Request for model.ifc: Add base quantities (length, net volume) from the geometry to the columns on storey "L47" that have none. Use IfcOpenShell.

First a look at what the model holds.

```python
import ifcopenshell
import ifcopenshell.util.element
import ifcopenshell.util.unit

model = ifcopenshell.open("model.ifc")
print(model.schema)
for unit_type in ("LENGTHUNIT", "AREAUNIT", "VOLUMEUNIT"):
    print(unit_type, ifcopenshell.util.unit.calculate_unit_scale(model, unit_type))
storey = next(s for s in model.by_type("IfcBuildingStorey") if s.Name == "L47")
columns = [e for e in ifcopenshell.util.element.get_decomposition(storey) if e.is_a("IfcColumn")]
for e in sorted(columns, key=lambda e: e.id()):
    print(e.id(), e.is_a(), e.Name, list(ifcopenshell.util.element.get_psets(e, qtos_only=True)), sep=" | ")
```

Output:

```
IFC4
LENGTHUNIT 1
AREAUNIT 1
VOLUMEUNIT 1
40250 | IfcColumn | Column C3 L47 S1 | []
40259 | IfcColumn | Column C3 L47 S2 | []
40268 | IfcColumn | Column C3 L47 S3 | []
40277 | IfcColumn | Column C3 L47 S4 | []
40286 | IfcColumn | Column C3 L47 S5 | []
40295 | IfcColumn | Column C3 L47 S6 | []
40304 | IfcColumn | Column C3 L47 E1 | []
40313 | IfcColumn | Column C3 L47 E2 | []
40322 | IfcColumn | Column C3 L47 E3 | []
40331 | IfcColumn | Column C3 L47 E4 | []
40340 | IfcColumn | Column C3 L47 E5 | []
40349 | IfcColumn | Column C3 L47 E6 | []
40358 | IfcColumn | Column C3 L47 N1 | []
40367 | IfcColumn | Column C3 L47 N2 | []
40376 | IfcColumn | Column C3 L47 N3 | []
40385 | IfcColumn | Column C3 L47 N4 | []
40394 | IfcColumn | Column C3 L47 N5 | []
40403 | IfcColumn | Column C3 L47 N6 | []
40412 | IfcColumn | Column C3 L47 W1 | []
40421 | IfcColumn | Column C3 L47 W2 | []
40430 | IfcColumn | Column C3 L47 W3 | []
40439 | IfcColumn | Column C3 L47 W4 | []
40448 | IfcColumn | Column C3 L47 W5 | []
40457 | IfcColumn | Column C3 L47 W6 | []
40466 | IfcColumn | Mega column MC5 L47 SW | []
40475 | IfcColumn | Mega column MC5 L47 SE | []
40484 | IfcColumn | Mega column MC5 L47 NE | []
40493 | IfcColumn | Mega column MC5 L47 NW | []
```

```python
import ifcopenshell
import ifcopenshell.api.pset
import ifcopenshell.geom
import ifcopenshell.util.element
import ifcopenshell.util.shape
import ifcopenshell.util.unit

model = ifcopenshell.open("model.ifc")
unit_scale = ifcopenshell.util.unit.calculate_unit_scale(model)
volume_scale = ifcopenshell.util.unit.calculate_unit_scale(model, "VOLUMEUNIT")
settings = ifcopenshell.geom.settings()

storey = next(s for s in model.by_type("IfcBuildingStorey") if s.Name == "L47")
columns = [e for e in ifcopenshell.util.element.get_decomposition(storey) if e.is_a("IfcColumn")]

for e in sorted(columns, key=lambda e: e.id()):
    if ifcopenshell.util.element.get_psets(e, qtos_only=True, should_inherit=False):
        continue
    # Geometry comes back in metres, in the element's own axes.
    shape = ifcopenshell.geom.create_shape(settings, e)
    values = {
        "Length": ifcopenshell.util.shape.get_z(shape.geometry) / unit_scale,
        "NetVolume": ifcopenshell.util.shape.get_volume(shape.geometry) / volume_scale,
    }
    qto = ifcopenshell.api.pset.add_qto(model, product=e, name="Qto_ColumnBaseQuantities")
    ifcopenshell.api.pset.edit_qto(model, qto=qto, properties=values)
    print(e.id(), {k: round(v, 3) for k, v in values.items()})

model.write("model_edited.ifc")
```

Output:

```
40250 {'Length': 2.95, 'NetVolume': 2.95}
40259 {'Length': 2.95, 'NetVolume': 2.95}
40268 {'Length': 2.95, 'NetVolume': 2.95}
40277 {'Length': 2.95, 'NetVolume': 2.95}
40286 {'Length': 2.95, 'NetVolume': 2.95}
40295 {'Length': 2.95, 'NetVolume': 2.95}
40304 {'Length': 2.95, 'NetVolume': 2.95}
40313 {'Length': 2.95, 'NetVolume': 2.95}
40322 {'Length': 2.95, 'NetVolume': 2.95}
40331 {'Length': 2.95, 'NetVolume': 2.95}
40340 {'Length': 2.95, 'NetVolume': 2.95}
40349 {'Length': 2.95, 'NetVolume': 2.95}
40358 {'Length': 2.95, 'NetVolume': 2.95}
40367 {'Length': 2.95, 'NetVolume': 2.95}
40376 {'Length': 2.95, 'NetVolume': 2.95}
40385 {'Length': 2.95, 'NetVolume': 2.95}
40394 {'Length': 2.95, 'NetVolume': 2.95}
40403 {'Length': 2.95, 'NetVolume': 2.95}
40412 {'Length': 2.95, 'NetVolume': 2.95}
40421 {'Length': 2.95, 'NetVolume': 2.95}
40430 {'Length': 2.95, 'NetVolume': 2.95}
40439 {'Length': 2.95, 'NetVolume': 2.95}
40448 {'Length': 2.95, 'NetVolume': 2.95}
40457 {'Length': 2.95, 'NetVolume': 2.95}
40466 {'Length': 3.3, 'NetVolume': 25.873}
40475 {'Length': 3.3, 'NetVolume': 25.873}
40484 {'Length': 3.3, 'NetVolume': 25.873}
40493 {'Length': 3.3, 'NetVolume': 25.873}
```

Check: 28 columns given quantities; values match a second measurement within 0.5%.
